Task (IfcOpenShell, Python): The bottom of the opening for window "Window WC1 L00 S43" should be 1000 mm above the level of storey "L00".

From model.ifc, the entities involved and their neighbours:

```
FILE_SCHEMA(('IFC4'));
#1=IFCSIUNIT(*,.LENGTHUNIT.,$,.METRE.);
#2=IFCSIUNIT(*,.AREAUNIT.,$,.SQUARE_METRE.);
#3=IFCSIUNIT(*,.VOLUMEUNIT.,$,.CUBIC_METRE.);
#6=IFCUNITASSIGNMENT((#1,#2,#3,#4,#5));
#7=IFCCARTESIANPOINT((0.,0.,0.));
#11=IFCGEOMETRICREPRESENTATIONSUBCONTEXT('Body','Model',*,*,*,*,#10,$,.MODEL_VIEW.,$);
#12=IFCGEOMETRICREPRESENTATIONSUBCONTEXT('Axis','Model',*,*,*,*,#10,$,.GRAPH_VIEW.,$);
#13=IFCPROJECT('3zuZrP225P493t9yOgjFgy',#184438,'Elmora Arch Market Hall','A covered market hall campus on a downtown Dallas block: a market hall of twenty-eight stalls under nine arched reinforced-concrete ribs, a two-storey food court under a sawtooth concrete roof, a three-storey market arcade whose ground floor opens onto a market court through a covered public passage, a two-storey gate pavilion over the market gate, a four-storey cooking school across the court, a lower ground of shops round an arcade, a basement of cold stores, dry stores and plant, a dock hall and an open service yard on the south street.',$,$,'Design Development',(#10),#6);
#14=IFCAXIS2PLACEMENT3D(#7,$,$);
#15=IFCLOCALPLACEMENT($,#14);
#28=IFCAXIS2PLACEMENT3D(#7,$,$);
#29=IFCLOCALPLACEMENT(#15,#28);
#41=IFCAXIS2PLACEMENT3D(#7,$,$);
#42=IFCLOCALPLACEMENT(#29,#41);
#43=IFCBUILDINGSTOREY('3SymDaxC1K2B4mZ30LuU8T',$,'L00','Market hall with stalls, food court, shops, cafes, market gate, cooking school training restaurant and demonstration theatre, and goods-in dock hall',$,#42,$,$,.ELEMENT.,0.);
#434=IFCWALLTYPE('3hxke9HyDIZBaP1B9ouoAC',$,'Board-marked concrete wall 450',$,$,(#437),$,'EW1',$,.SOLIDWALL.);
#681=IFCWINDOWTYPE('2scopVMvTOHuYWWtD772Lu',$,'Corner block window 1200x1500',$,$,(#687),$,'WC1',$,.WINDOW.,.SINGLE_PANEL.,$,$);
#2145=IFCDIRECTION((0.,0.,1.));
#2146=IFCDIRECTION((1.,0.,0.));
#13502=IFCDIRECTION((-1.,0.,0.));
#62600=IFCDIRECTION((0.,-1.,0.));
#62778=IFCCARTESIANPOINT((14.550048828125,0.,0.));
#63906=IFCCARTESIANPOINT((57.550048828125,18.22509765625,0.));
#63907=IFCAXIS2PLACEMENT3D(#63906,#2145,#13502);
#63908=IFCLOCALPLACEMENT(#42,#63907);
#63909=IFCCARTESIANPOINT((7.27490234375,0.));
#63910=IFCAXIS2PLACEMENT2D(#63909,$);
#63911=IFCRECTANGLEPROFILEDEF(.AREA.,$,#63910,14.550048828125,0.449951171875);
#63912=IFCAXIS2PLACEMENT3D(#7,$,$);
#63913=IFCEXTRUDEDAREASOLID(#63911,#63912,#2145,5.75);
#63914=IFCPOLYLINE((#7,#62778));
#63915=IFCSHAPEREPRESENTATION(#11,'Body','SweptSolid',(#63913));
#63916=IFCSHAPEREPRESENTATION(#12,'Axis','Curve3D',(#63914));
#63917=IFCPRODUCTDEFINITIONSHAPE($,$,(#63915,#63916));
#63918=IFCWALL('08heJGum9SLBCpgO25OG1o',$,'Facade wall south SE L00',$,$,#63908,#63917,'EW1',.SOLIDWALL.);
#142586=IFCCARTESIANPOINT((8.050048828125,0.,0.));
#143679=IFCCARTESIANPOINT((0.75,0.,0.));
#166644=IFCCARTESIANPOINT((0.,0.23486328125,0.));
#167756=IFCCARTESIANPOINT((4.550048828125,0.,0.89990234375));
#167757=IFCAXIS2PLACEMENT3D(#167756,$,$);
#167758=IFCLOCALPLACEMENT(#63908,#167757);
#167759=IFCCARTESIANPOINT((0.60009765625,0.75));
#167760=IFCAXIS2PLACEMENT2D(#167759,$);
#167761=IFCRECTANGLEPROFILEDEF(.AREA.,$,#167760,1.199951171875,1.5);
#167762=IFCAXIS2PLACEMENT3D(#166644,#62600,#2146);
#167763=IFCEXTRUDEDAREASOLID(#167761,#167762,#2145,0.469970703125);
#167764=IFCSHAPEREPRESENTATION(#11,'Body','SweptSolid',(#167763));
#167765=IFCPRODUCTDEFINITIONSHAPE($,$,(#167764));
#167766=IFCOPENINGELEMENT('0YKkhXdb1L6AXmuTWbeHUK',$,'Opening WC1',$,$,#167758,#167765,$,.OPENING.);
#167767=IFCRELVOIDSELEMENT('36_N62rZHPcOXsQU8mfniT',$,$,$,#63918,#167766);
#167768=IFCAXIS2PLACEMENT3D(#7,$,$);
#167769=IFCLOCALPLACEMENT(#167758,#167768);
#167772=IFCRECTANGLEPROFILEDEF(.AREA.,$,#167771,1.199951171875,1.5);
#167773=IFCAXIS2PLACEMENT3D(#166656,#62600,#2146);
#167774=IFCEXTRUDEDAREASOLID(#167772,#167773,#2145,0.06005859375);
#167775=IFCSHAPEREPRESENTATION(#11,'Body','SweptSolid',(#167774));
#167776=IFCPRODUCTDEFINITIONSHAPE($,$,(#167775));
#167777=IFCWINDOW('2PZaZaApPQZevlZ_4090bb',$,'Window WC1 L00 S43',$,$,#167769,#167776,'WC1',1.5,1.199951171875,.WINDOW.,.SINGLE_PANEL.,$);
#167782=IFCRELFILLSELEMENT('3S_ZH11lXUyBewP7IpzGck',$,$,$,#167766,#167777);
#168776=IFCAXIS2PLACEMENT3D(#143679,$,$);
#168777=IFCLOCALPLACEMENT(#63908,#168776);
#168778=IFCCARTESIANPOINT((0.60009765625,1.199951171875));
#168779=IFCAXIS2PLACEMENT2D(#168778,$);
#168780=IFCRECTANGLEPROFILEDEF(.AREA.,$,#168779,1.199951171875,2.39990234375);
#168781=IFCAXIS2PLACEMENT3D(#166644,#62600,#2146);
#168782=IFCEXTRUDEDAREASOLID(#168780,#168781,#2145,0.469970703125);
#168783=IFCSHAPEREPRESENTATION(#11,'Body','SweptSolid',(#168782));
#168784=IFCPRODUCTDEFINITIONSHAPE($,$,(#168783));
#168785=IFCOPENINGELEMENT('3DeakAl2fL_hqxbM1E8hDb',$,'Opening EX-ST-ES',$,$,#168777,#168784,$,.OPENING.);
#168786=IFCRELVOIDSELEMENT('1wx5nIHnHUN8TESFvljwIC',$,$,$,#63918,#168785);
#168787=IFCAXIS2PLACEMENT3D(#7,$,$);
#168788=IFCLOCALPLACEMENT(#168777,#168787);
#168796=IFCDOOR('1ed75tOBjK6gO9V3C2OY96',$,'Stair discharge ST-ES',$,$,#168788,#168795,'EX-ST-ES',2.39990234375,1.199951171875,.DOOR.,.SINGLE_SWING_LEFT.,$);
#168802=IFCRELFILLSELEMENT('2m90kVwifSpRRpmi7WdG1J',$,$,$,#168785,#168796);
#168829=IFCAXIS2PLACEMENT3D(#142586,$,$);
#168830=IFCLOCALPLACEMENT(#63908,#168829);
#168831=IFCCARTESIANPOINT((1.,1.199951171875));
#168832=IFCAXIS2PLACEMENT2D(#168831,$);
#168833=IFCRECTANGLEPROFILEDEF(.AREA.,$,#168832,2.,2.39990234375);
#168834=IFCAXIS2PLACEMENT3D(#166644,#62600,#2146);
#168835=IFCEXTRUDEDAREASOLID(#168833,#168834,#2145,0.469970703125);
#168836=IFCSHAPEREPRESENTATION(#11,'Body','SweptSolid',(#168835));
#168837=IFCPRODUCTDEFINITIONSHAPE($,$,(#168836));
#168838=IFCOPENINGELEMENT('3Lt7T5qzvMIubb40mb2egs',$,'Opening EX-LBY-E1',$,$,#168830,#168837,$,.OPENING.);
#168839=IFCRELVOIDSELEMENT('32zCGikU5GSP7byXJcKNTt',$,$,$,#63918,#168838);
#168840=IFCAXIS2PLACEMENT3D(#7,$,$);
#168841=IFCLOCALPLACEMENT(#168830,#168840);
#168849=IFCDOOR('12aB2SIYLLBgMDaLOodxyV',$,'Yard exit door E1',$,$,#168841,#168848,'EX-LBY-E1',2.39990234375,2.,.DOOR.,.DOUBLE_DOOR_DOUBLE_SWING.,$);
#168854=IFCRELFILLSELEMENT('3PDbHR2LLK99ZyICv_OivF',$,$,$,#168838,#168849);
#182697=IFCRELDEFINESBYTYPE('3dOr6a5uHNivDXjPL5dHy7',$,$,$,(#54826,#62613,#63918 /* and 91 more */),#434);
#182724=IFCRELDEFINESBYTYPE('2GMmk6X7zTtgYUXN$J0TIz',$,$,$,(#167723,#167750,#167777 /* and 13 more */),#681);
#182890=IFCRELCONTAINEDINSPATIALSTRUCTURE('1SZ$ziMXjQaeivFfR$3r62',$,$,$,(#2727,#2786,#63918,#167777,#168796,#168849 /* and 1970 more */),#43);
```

```python
import numpy as np
import ifcopenshell
import ifcopenshell.api.geometry
import ifcopenshell.geom
import ifcopenshell.util.element
import ifcopenshell.util.placement
import ifcopenshell.util.shape
import ifcopenshell.util.unit

model = ifcopenshell.open("model.ifc")
unit_scale = ifcopenshell.util.unit.calculate_unit_scale(model)

window = model.by_id(167777)
opening = window.FillsVoids[0].RelatingOpeningElement
storey = ifcopenshell.util.element.get_container(window, ifc_class="IfcBuildingStorey")
level = ifcopenshell.util.placement.get_local_placement(storey.ObjectPlacement)[2, 3]

# The opening's origin need not be at the sill, so measure its lowest point.
shape = ifcopenshell.geom.create_shape(ifcopenshell.geom.settings(), opening)
bottom = ifcopenshell.util.shape.get_shape_bottom_elevation(shape, shape.geometry) / unit_scale
dz = level + 1.0 - bottom

shift = np.array([0.0, 0.0, dz])
# The window is placed relative to its opening, so it follows when the opening moves.
matrix = ifcopenshell.util.placement.get_local_placement(opening.ObjectPlacement)
matrix[:3, 3] += shift
ifcopenshell.api.geometry.edit_object_placement(
    model, product=opening, matrix=matrix, is_si=False, should_transform_children=True
)

print(f"moved by {dz * unit_scale:+.3f} m")

model.write("model_edited.ifc")
```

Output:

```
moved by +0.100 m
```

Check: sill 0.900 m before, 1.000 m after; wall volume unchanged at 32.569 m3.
